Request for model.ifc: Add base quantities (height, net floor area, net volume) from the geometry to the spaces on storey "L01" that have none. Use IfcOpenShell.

First a look at what the model holds.

```python
import ifcopenshell
import ifcopenshell.util.element
import ifcopenshell.util.unit

model = ifcopenshell.open("model.ifc")
print(model.schema)
for unit_type in ("LENGTHUNIT", "AREAUNIT", "VOLUMEUNIT"):
    print(unit_type, ifcopenshell.util.unit.calculate_unit_scale(model, unit_type))
storey = next(s for s in model.by_type("IfcBuildingStorey") if s.Name == "L01")
spaces = [e for e in ifcopenshell.util.element.get_decomposition(storey) if e.is_a("IfcSpace")]
for e in sorted(spaces, key=lambda e: e.id()):
    print(e.id(), e.is_a(), e.Name, list(ifcopenshell.util.element.get_psets(e, qtos_only=True)), sep=" | ")
```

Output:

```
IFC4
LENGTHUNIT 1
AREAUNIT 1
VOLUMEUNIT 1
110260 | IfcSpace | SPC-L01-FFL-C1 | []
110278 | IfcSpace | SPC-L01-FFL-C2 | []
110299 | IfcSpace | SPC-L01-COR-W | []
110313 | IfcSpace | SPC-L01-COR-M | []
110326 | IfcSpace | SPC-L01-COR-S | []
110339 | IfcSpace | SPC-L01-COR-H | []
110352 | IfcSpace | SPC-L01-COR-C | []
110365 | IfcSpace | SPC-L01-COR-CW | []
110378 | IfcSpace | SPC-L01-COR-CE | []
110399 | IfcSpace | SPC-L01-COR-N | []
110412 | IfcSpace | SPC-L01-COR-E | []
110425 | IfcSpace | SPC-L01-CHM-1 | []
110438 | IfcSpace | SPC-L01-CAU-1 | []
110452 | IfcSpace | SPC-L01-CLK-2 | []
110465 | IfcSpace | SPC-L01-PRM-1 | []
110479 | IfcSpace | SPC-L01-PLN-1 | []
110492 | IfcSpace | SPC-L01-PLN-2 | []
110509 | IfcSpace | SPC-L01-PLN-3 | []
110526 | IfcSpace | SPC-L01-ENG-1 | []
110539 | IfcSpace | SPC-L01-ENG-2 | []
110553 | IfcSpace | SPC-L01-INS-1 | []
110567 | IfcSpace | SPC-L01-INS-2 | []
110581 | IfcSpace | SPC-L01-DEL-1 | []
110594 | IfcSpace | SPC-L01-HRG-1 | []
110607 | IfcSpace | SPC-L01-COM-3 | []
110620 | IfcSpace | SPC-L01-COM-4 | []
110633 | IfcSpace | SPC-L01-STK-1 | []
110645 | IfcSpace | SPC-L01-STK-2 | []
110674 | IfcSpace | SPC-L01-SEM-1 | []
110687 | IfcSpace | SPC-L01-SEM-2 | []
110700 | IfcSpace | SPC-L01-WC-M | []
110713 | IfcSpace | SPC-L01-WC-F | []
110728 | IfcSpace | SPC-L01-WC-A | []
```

```python
import ifcopenshell
import ifcopenshell.api.pset
import ifcopenshell.geom
import ifcopenshell.util.element
import ifcopenshell.util.shape
import ifcopenshell.util.unit

model = ifcopenshell.open("model.ifc")
unit_scale = ifcopenshell.util.unit.calculate_unit_scale(model)
area_scale = ifcopenshell.util.unit.calculate_unit_scale(model, "AREAUNIT")
volume_scale = ifcopenshell.util.unit.calculate_unit_scale(model, "VOLUMEUNIT")
settings = ifcopenshell.geom.settings()

storey = next(s for s in model.by_type("IfcBuildingStorey") if s.Name == "L01")
spaces = [e for e in ifcopenshell.util.element.get_decomposition(storey) if e.is_a("IfcSpace")]

for e in sorted(spaces, key=lambda e: e.id()):
    if ifcopenshell.util.element.get_psets(e, qtos_only=True, should_inherit=False):
        continue
    # Geometry comes back in metres, in the element's own axes.
    shape = ifcopenshell.geom.create_shape(settings, e)
    values = {
        "Height": ifcopenshell.util.shape.get_z(shape.geometry) / unit_scale,
        "NetFloorArea": ifcopenshell.util.shape.get_footprint_area(shape.geometry) / area_scale,
        "NetVolume": ifcopenshell.util.shape.get_volume(shape.geometry) / volume_scale,
    }
    qto = ifcopenshell.api.pset.add_qto(model, product=e, name="Qto_SpaceBaseQuantities")
    ifcopenshell.api.pset.edit_qto(model, qto=qto, properties=values)
    print(e.id(), {k: round(v, 3) for k, v in values.items()})

model.write("model_v2.ifc")
```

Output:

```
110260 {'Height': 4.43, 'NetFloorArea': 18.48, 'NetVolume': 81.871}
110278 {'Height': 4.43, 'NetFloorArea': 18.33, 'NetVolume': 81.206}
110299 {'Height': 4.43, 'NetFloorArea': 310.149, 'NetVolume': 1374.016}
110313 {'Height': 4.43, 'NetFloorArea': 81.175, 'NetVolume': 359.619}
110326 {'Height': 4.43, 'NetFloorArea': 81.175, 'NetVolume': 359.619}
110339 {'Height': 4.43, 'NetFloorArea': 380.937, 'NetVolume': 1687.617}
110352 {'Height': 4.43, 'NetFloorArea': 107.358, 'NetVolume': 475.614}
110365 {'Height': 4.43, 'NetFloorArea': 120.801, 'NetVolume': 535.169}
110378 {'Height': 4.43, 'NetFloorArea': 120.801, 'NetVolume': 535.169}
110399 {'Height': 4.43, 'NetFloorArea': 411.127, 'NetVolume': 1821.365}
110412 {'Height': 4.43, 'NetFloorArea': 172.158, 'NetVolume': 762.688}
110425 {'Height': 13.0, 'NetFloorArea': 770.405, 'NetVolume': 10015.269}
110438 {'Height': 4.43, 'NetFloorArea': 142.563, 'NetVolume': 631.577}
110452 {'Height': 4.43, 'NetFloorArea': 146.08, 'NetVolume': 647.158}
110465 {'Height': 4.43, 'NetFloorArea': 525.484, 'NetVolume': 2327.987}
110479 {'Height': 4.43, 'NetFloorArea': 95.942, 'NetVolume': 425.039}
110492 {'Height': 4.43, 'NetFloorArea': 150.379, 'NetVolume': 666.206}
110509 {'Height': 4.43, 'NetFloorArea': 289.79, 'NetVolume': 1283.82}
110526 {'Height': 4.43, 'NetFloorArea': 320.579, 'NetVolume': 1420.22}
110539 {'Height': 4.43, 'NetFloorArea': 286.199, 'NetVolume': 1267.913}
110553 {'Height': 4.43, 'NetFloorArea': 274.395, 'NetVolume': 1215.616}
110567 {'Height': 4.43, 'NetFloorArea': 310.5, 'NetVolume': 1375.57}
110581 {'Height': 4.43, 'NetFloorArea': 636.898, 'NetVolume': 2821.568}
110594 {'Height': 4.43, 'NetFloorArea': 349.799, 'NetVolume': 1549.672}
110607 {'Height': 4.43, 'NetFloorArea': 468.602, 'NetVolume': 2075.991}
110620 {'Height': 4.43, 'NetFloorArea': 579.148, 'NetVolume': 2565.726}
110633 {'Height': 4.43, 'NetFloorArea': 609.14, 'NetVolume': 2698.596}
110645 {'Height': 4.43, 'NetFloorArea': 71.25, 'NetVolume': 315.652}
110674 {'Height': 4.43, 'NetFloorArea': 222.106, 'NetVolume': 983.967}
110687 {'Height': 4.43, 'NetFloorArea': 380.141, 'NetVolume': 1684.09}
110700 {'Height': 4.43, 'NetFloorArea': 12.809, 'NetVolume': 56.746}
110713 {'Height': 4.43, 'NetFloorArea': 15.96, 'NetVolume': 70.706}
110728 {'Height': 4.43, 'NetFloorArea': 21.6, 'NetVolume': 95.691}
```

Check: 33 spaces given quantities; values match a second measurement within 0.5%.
